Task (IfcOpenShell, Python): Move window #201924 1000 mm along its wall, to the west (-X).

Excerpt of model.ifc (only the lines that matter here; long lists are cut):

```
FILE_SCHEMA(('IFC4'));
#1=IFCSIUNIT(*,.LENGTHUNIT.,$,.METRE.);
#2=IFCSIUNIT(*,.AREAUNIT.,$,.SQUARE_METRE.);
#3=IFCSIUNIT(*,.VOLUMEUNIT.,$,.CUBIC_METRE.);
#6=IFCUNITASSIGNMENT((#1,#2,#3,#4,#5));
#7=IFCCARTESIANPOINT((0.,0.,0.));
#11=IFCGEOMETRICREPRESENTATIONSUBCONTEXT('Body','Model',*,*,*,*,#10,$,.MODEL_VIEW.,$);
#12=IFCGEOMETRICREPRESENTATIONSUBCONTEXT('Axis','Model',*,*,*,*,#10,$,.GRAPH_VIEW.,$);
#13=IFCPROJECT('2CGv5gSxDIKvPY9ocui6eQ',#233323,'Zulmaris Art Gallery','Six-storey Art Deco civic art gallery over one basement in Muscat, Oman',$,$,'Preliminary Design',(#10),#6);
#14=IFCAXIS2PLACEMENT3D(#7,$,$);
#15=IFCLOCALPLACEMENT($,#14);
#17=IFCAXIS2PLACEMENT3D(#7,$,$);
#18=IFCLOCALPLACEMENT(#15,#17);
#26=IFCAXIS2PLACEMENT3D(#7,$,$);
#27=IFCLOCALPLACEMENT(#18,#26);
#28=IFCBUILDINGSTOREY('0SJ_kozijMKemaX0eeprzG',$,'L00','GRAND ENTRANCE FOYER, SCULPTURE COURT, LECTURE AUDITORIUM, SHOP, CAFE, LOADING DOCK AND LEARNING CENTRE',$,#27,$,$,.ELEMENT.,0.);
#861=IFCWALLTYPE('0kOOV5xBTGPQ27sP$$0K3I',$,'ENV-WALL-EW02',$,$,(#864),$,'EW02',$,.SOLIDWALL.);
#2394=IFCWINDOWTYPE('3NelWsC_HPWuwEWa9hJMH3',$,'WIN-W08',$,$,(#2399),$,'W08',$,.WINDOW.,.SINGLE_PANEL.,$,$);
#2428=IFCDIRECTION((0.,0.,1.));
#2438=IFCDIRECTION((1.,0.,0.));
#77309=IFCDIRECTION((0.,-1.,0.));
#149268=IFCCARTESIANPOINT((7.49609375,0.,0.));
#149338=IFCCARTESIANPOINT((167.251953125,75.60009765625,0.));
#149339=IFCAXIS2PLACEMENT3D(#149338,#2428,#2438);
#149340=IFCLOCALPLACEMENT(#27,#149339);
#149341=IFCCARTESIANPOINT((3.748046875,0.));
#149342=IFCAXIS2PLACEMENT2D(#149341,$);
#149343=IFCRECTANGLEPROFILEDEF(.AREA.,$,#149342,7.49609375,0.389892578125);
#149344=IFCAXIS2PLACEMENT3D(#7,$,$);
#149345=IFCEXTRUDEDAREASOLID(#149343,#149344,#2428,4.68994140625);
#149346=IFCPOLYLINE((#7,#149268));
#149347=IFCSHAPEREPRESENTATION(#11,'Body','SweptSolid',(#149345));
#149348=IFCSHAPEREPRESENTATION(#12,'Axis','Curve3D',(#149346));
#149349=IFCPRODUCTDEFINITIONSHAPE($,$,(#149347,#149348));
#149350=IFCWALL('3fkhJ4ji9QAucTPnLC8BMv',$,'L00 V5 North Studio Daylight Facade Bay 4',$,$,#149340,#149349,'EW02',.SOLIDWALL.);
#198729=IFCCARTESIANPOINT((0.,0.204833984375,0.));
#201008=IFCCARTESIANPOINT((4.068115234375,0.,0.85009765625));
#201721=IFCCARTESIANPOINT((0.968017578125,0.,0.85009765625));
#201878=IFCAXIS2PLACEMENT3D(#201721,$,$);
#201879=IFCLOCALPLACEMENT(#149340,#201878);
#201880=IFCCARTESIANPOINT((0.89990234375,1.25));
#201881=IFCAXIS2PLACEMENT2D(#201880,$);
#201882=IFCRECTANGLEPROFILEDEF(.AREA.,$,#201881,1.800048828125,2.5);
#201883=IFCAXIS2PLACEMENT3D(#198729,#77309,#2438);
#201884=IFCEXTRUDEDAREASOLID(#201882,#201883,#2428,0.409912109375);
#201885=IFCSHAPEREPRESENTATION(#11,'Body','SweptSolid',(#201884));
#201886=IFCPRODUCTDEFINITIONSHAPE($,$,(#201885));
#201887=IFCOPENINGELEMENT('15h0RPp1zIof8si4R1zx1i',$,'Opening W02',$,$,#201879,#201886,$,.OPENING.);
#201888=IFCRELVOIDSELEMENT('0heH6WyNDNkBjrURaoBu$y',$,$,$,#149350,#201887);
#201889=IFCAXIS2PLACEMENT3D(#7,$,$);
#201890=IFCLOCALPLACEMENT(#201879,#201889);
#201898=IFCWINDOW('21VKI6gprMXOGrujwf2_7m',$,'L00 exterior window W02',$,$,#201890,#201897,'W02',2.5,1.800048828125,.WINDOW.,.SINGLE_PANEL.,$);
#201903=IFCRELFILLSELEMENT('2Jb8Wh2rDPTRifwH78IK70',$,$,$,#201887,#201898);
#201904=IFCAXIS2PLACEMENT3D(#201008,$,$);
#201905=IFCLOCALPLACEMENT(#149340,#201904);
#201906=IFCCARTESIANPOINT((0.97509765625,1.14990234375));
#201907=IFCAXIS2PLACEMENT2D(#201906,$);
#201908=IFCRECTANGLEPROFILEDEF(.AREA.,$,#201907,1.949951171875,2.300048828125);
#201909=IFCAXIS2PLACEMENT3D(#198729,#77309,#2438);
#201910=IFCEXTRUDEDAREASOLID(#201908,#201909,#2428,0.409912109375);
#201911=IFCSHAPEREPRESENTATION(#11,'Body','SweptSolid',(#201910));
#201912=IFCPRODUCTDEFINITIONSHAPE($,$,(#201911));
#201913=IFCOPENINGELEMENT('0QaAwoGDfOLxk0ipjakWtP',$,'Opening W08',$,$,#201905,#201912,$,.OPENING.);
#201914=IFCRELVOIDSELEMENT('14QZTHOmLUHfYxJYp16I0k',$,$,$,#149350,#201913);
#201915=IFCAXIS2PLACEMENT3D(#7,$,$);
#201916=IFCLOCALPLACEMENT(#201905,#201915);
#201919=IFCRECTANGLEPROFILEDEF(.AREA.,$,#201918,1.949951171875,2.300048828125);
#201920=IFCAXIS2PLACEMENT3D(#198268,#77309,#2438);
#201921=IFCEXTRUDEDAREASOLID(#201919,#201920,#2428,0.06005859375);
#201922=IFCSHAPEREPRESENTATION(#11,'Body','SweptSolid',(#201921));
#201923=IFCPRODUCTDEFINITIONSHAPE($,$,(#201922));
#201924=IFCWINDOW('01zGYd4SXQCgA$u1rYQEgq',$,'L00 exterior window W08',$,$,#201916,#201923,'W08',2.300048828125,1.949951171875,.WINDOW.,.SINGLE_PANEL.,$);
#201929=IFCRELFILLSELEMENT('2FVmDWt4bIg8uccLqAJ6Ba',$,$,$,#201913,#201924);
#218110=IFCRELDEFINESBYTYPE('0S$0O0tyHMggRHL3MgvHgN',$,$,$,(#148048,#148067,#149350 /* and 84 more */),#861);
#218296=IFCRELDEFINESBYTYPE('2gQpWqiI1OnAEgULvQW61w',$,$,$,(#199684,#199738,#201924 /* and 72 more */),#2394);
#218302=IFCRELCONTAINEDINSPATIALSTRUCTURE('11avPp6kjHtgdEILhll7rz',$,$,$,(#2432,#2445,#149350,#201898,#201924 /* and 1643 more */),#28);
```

```python
import ifcopenshell
import ifcopenshell.api.geometry
import ifcopenshell.util.placement
import ifcopenshell.util.unit

model = ifcopenshell.open("model.ifc")
unit_scale = ifcopenshell.util.unit.calculate_unit_scale(model)

window = model.by_guid("01zGYd4SXQCgA$u1rYQEgq")
opening = window.FillsVoids[0].RelatingOpeningElement
wall = opening.VoidsElements[0].RelatingBuildingElement

wall_matrix = ifcopenshell.util.placement.get_local_placement(wall.ObjectPlacement)
shift = wall_matrix[:3, 0] * -1 / unit_scale
before = ifcopenshell.util.placement.get_local_placement(window.ObjectPlacement)[:3, 3].copy()

# The window is placed relative to its opening, so it follows when the opening moves.
matrix = ifcopenshell.util.placement.get_local_placement(opening.ObjectPlacement)
matrix[:3, 3] += shift
ifcopenshell.api.geometry.edit_object_placement(
    model, product=opening, matrix=matrix, is_si=False, should_transform_children=True
)

after = ifcopenshell.util.placement.get_local_placement(window.ObjectPlacement)[:3, 3]
print("window moved by", (after - before).round(3) + 0.0)

model.write("model_rev.ifc")
```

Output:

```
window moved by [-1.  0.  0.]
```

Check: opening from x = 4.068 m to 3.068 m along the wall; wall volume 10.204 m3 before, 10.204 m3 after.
